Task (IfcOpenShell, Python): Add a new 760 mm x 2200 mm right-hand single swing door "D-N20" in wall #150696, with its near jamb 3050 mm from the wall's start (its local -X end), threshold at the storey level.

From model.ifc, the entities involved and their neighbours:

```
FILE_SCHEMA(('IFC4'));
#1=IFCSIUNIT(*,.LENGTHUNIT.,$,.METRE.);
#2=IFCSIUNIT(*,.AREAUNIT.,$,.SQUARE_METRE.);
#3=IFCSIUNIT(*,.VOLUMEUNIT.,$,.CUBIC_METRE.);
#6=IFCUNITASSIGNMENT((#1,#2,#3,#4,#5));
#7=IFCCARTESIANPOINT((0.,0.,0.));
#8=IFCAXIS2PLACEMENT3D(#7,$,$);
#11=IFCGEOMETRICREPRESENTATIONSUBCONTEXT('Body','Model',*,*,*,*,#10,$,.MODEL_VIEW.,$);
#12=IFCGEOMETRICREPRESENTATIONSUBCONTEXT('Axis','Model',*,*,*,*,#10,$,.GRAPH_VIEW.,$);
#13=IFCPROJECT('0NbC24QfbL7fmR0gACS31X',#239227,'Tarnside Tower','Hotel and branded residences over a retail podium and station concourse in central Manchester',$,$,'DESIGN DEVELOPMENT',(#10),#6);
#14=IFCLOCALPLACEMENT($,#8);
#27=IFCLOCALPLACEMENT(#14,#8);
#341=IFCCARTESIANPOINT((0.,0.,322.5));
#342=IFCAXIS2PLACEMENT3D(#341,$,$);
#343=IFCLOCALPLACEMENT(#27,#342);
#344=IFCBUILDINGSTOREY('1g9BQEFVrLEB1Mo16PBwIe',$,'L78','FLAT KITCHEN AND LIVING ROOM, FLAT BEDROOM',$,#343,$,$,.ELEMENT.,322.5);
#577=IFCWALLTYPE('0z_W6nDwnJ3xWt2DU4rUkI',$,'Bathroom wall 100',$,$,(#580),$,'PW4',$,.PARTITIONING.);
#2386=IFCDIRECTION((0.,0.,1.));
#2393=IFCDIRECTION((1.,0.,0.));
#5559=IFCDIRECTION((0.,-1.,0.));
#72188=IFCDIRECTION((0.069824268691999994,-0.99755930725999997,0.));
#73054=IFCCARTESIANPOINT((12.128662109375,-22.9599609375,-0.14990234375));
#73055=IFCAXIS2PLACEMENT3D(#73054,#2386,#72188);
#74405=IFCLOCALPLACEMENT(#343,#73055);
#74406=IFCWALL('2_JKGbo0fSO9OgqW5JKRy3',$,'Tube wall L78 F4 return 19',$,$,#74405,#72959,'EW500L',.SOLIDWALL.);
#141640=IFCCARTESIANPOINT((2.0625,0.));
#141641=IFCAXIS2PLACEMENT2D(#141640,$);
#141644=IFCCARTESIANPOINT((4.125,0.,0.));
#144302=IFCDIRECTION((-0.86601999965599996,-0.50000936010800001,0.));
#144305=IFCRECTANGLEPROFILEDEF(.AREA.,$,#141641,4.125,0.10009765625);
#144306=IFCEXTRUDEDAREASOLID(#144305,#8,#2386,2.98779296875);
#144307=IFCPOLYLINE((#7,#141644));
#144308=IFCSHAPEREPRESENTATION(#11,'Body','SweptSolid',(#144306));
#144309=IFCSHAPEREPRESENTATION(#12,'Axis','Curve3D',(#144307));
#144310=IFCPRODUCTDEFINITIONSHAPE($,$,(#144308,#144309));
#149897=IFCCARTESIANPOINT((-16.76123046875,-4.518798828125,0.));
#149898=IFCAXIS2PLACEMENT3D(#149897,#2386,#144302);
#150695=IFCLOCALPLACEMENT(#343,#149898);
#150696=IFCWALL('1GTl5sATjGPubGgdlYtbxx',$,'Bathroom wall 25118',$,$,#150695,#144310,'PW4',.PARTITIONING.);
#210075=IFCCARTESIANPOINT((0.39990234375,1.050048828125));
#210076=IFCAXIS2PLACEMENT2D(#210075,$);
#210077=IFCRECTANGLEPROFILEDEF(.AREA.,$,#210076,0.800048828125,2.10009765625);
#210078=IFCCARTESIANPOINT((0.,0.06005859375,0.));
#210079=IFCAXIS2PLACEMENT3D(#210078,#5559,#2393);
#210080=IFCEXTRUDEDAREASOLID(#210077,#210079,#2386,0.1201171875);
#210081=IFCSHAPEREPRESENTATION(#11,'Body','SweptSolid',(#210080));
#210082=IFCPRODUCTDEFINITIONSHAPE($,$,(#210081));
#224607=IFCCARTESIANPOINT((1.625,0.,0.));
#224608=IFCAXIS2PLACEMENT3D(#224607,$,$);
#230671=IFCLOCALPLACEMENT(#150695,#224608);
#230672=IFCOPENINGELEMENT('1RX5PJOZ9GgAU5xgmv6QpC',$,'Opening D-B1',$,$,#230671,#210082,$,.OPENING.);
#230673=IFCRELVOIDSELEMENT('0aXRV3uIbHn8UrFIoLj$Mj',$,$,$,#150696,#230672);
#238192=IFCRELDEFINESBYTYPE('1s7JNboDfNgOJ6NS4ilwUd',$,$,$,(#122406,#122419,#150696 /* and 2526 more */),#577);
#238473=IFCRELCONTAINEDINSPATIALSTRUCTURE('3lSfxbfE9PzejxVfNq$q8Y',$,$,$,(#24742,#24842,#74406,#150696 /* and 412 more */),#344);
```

```python
import numpy as np
import ifcopenshell
import ifcopenshell.api.feature
import ifcopenshell.api.geometry
import ifcopenshell.api.root
import ifcopenshell.api.spatial
import ifcopenshell.geom
import ifcopenshell.util.element
import ifcopenshell.util.placement
import ifcopenshell.util.representation
import ifcopenshell.util.shape
import ifcopenshell.util.unit

model = ifcopenshell.open("model.ifc")
unit_scale = ifcopenshell.util.unit.calculate_unit_scale(model)
settings = ifcopenshell.geom.settings()


def volume(element):
    """Net volume in cubic metres, openings subtracted."""
    shape = ifcopenshell.geom.create_shape(settings, element)
    return ifcopenshell.util.shape.get_volume(shape.geometry)


wall = model.by_guid("1GTl5sATjGPubGgdlYtbxx")
storey = ifcopenshell.util.element.get_container(wall, ifc_class="IfcBuildingStorey")
context = ifcopenshell.util.representation.get_context(model, "Model", "Body", "MODEL_VIEW")
before = volume(wall)

width, height, from_end, sill = 0.76, 2.2, 3.05, 0.0  # metres

# The wall runs along its own X axis, and the end named is its -X end.
wall_shape = ifcopenshell.geom.create_shape(settings, wall)
x, y, z = ifcopenshell.util.shape.get_vertices(wall_shape.geometry).T
start = x.min() + from_end
face, thickness = float(y.min()), float(y.max() - y.min())
wall_matrix = ifcopenshell.util.placement.get_local_placement(wall.ObjectPlacement)
level = ifcopenshell.util.placement.get_local_placement(storey.ObjectPlacement)[2, 3]


def in_wall(x, y):
    """Placement at x, y metres in the wall's axes, at sill height."""
    matrix = wall_matrix.copy()
    matrix[:, 3] = wall_matrix @ np.array([x / unit_scale, y / unit_scale, 0.0, 1.0])
    matrix[2, 3] = level + sill / unit_scale
    return matrix


# Opening: a box that overshoots both wall faces by 50 mm.
opening = ifcopenshell.api.root.create_entity(model, ifc_class="IfcOpeningElement", predefined_type="OPENING")
box = ifcopenshell.api.geometry.add_wall_representation(
    model, context=context, length=width, height=height, thickness=thickness + 0.1
)
ifcopenshell.api.geometry.assign_representation(model, product=opening, representation=box)
ifcopenshell.api.geometry.edit_object_placement(model, product=opening, matrix=in_wall(start, face - 0.05), is_si=False)
ifcopenshell.api.feature.add_feature(model, feature=opening, element=wall)

door = ifcopenshell.api.root.create_entity(model, ifc_class="IfcDoor", name="D-N20", predefined_type="DOOR")
door.OverallWidth, door.OverallHeight = width / unit_scale, height / unit_scale
door.OperationType = "SINGLE_SWING_RIGHT"
body = ifcopenshell.api.geometry.add_door_representation(
    model,
    context=context,
    overall_width=door.OverallWidth,
    overall_height=door.OverallHeight,
    operation_type="SINGLE_SWING_RIGHT",
    lining_properties={"LiningDepth": thickness / unit_scale, "ThresholdDepth": thickness / unit_scale},
)
ifcopenshell.api.geometry.assign_representation(model, product=door, representation=body)
ifcopenshell.api.spatial.assign_container(model, products=[door], relating_structure=storey)
ifcopenshell.api.feature.add_filling(model, opening=opening, element=door)

# The lining spans the wall, so the door starts at the wall face.
ifcopenshell.api.geometry.edit_object_placement(model, product=door, matrix=in_wall(start, face), is_si=False)

after = volume(wall)

print(f"wall volume {before:.3f} -> {after:.3f} m3")

model.write("model_rev.ifc")
```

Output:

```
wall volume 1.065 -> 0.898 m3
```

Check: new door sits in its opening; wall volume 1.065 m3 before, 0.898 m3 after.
